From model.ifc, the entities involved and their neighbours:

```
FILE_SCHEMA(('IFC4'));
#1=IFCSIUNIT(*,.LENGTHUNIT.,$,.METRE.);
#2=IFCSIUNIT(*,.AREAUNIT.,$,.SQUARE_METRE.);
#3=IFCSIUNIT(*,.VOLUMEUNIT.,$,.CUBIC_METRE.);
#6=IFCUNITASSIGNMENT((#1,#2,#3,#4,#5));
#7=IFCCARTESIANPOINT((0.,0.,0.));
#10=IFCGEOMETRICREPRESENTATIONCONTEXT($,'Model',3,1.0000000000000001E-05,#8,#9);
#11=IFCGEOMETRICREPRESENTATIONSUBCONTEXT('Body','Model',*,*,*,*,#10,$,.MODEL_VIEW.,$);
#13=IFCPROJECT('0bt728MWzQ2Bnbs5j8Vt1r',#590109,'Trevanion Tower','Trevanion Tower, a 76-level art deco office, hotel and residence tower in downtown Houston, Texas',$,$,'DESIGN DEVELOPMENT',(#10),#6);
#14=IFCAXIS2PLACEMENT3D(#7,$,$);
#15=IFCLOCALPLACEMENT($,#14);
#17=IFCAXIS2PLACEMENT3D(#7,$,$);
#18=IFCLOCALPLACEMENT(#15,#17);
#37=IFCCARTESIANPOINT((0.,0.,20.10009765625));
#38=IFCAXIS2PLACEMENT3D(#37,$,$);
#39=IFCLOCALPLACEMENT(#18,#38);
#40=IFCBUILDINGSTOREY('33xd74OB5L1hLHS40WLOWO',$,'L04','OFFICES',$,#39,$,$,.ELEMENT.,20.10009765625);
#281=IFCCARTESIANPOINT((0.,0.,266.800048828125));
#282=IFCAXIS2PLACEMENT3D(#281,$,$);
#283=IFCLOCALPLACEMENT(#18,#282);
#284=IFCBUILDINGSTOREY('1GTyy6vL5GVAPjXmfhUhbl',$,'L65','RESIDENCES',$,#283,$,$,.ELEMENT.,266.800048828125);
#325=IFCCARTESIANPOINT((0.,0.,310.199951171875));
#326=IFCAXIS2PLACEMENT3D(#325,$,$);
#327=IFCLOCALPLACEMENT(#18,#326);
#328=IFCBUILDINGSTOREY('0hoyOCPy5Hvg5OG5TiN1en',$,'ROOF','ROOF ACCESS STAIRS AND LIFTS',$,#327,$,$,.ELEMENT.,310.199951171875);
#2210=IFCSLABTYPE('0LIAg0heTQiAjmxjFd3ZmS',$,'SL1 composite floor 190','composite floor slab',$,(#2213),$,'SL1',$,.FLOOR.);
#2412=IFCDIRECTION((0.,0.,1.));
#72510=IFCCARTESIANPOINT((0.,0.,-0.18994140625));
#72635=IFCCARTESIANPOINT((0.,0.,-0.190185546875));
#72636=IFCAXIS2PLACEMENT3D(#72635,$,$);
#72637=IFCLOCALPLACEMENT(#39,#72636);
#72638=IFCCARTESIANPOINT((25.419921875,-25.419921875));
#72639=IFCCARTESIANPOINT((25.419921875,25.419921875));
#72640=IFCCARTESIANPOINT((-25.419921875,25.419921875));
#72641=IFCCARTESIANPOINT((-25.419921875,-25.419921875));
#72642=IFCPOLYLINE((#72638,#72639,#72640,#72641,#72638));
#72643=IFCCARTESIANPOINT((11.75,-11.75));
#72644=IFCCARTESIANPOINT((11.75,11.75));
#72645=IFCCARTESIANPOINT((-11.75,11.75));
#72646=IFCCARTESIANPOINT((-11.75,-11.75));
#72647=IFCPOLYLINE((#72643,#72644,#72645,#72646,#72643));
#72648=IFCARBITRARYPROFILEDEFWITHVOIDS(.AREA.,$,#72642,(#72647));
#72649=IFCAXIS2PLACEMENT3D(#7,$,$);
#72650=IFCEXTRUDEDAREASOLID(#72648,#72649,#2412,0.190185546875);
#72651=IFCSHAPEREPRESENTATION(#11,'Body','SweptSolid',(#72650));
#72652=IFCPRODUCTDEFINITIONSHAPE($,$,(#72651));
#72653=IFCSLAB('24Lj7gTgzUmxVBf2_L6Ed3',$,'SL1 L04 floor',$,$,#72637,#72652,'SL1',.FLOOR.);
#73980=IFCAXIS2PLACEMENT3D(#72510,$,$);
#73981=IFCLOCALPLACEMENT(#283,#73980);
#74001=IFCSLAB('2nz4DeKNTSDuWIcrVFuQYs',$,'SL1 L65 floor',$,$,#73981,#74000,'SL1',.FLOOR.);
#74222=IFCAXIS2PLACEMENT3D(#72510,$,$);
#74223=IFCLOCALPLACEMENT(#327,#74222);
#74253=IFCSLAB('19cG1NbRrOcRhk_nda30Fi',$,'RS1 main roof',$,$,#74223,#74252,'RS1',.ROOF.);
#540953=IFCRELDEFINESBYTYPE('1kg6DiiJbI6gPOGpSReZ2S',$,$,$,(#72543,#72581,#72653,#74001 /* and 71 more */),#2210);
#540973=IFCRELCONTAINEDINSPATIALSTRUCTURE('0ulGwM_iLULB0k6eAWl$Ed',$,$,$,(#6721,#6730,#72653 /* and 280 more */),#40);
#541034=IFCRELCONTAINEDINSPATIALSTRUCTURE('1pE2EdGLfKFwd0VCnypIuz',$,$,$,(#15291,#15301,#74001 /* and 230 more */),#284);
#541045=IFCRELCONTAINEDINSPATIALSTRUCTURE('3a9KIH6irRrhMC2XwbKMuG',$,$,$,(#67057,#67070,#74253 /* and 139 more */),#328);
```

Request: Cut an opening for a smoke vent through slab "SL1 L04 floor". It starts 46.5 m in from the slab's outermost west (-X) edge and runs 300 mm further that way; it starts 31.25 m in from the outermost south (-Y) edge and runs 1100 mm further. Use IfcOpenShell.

```python
import numpy as np
import ifcopenshell
import ifcopenshell.api.feature
import ifcopenshell.api.geometry
import ifcopenshell.api.root
import ifcopenshell.geom
import ifcopenshell.util.placement
import ifcopenshell.util.representation
import ifcopenshell.util.shape
import ifcopenshell.util.unit

model = ifcopenshell.open("model.ifc")
unit_scale = ifcopenshell.util.unit.calculate_unit_scale(model)
settings = ifcopenshell.geom.settings()


def volume(element):
    """Net volume in cubic metres, openings subtracted."""
    shape = ifcopenshell.geom.create_shape(settings, element)
    return ifcopenshell.util.shape.get_volume(shape.geometry)


slab = model.by_guid("24Lj7gTgzUmxVBf2_L6Ed3")
before = volume(slab)

# Extent in the slab's own axes, in metres. The edges named are its -X and -Y sides.
slab_shape = ifcopenshell.geom.create_shape(settings, slab)
vertices = ifcopenshell.util.shape.get_vertices(slab_shape.geometry)
x_min, y_min, bottom = vertices.min(axis=0)
top = vertices[:, 2].max()

opening = ifcopenshell.api.root.create_entity(model, ifc_class="IfcOpeningElement", name="Smoke vent opening", predefined_type="OPENING")
context = ifcopenshell.util.representation.get_context(model, "Model", "Body", "MODEL_VIEW")
width, depth = 0.3, 1.1
outline = [(0.0, 0.0), (width, 0.0), (width, depth), (0.0, depth), (0.0, 0.0)]
# Overshoot both faces by 50 mm so the cut is clean.
shape = ifcopenshell.api.geometry.add_slab_representation(
    model, context=context, depth=top - bottom + 0.1, polyline=outline
)
ifcopenshell.api.geometry.assign_representation(model, product=opening, representation=shape)

matrix = ifcopenshell.util.placement.get_local_placement(slab.ObjectPlacement)
matrix[:, 3] = matrix @ np.append(np.array([x_min + 46.5, y_min + 31.25, bottom - 0.05]) / unit_scale, 1.0)
ifcopenshell.api.geometry.edit_object_placement(model, product=opening, matrix=matrix, is_si=False)
ifcopenshell.api.feature.add_feature(model, feature=opening, element=slab)

after = volume(slab)

print(f"slab volume {before:.3f} -> {after:.3f} m3")

model.write("model_edited.ifc")
```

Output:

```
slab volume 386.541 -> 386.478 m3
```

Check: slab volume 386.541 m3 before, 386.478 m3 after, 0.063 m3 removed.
